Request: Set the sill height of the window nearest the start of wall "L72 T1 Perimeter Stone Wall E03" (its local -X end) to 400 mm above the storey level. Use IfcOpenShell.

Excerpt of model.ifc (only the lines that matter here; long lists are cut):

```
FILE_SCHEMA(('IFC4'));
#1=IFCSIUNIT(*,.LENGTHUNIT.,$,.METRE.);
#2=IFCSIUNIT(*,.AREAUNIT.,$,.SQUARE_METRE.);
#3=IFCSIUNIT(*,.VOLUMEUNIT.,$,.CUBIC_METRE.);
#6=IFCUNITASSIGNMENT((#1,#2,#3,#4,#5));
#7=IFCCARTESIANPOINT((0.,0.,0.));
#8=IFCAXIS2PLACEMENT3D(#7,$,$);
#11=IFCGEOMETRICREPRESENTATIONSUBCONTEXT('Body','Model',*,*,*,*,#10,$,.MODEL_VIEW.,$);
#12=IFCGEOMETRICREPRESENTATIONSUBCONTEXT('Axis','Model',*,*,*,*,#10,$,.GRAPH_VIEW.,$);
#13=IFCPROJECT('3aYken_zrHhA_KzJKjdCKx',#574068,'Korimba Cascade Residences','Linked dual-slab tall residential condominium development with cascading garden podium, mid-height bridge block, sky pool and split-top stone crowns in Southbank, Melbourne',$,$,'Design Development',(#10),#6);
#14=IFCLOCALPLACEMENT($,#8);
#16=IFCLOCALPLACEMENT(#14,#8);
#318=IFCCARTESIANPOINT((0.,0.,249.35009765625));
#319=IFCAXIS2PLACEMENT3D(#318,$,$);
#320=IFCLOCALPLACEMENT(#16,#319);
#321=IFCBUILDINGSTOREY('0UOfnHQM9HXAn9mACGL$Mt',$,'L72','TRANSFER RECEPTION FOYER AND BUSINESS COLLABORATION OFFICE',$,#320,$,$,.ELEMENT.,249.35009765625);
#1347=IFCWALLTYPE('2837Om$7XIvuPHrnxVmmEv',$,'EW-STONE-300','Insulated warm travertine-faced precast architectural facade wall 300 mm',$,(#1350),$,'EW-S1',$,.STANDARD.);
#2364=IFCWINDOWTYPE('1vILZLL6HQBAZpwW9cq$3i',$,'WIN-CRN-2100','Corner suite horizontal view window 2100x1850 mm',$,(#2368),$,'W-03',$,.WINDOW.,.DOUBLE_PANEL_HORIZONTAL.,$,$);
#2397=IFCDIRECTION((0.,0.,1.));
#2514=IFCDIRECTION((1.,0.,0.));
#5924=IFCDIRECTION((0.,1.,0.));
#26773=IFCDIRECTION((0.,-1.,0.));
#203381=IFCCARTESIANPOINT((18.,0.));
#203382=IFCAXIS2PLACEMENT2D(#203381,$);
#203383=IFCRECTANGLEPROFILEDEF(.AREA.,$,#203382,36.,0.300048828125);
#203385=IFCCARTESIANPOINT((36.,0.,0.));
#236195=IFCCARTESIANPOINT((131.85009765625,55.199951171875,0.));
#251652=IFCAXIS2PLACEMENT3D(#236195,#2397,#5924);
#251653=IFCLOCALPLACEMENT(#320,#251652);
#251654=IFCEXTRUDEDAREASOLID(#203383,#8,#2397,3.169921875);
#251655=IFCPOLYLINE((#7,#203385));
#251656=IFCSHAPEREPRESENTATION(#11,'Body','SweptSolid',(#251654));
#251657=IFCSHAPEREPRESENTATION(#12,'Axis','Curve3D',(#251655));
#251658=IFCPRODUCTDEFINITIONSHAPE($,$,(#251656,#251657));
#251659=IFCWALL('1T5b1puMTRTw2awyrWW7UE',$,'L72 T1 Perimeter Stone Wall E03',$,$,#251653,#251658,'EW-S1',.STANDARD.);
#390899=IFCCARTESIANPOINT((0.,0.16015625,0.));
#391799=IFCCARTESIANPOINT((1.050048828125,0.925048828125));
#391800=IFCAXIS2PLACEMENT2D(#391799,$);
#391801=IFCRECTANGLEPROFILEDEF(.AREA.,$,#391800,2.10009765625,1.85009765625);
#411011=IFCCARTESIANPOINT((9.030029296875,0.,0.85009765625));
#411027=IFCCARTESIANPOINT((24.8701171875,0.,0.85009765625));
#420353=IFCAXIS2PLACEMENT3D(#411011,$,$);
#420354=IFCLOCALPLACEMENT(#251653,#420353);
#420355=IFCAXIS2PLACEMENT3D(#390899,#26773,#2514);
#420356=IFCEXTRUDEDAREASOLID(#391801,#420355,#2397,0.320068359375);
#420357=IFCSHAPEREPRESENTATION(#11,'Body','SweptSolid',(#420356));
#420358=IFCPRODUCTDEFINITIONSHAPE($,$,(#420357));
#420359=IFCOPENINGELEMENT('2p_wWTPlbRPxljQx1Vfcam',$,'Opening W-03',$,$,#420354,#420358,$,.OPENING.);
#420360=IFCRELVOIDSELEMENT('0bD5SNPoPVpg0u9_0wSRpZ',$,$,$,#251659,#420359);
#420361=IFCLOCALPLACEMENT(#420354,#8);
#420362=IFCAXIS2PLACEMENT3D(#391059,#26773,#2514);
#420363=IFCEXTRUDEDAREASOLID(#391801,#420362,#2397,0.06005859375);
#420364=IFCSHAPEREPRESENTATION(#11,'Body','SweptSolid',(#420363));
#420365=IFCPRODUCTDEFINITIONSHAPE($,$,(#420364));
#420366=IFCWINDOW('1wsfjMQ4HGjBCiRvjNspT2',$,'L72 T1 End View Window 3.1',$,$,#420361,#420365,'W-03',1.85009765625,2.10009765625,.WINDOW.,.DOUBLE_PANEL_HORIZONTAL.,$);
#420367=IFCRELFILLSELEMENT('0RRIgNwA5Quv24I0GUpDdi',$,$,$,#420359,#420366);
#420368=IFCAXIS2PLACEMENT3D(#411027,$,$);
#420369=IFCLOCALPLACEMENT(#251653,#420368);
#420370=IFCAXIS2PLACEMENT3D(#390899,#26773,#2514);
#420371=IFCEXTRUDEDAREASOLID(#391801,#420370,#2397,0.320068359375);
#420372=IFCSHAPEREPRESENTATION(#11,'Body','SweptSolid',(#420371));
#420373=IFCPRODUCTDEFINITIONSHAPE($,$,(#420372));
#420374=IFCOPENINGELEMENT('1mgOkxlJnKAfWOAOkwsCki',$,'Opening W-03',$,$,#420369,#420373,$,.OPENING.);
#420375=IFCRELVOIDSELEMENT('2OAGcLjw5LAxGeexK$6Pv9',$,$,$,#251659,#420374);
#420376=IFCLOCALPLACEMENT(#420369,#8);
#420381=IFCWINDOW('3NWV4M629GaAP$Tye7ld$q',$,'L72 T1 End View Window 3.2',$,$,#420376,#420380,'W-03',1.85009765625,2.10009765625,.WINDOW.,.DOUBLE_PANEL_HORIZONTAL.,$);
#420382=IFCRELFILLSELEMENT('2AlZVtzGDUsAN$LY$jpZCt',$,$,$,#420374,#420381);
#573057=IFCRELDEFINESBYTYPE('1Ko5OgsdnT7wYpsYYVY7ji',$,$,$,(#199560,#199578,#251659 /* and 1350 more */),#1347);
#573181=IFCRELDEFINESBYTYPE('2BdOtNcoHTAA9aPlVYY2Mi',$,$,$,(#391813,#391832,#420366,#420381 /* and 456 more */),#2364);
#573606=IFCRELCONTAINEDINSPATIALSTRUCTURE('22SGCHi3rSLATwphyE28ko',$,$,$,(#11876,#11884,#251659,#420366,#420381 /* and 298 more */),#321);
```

```python
import numpy as np
import ifcopenshell
import ifcopenshell.api.geometry
import ifcopenshell.geom
import ifcopenshell.util.element
import ifcopenshell.util.placement
import ifcopenshell.util.shape
import ifcopenshell.util.unit

model = ifcopenshell.open("model.ifc")
unit_scale = ifcopenshell.util.unit.calculate_unit_scale(model)

window = model.by_guid("1wsfjMQ4HGjBCiRvjNspT2")
opening = window.FillsVoids[0].RelatingOpeningElement
storey = ifcopenshell.util.element.get_container(window, ifc_class="IfcBuildingStorey")
level = ifcopenshell.util.placement.get_local_placement(storey.ObjectPlacement)[2, 3]

# The opening's origin need not be at the sill, so measure its lowest point.
shape = ifcopenshell.geom.create_shape(ifcopenshell.geom.settings(), opening)
bottom = ifcopenshell.util.shape.get_shape_bottom_elevation(shape, shape.geometry) / unit_scale
dz = level + 0.4 - bottom

shift = np.array([0.0, 0.0, dz])
# The window is placed relative to its opening, so it follows when the opening moves.
matrix = ifcopenshell.util.placement.get_local_placement(opening.ObjectPlacement)
matrix[:3, 3] += shift
ifcopenshell.api.geometry.edit_object_placement(
    model, product=opening, matrix=matrix, is_si=False, should_transform_children=True
)

print(f"moved by {dz * unit_scale:+.3f} m")

model.write("model_edited.ifc")
```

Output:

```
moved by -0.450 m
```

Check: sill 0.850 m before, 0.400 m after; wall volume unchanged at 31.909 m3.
